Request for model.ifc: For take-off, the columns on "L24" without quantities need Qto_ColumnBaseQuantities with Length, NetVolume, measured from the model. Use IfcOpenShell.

First a look at what the model holds.

```python
import ifcopenshell
import ifcopenshell.util.element
import ifcopenshell.util.unit

model = ifcopenshell.open("model.ifc")
print(model.schema)
for unit_type in ("LENGTHUNIT", "AREAUNIT", "VOLUMEUNIT"):
    print(unit_type, ifcopenshell.util.unit.calculate_unit_scale(model, unit_type))
storey = next(s for s in model.by_type("IfcBuildingStorey") if s.Name == "L24")
columns = [e for e in ifcopenshell.util.element.get_decomposition(storey) if e.is_a("IfcColumn")]
for e in sorted(columns, key=lambda e: e.id()):
    print(e.id(), e.is_a(), e.Name, list(ifcopenshell.util.element.get_psets(e, qtos_only=True)), sep=" | ")
```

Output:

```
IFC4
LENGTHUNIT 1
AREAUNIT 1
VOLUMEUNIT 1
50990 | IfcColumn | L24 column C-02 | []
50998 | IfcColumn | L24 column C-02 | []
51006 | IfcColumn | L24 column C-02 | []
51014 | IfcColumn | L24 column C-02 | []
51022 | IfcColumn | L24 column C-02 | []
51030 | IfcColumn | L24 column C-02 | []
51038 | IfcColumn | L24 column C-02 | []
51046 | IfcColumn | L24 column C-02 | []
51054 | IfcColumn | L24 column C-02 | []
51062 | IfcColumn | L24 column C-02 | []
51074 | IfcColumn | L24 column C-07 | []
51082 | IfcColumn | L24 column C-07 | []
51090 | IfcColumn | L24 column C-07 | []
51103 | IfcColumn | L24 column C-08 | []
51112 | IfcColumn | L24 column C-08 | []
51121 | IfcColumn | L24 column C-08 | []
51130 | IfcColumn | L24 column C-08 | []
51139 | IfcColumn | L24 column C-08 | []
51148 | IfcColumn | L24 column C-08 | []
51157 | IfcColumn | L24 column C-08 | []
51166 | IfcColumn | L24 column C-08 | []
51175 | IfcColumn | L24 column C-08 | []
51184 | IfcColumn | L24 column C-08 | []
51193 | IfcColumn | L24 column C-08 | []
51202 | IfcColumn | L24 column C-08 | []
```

```python
import ifcopenshell
import ifcopenshell.api.pset
import ifcopenshell.geom
import ifcopenshell.util.element
import ifcopenshell.util.shape
import ifcopenshell.util.unit

model = ifcopenshell.open("model.ifc")
unit_scale = ifcopenshell.util.unit.calculate_unit_scale(model)
volume_scale = ifcopenshell.util.unit.calculate_unit_scale(model, "VOLUMEUNIT")
settings = ifcopenshell.geom.settings()

storey = next(s for s in model.by_type("IfcBuildingStorey") if s.Name == "L24")
columns = [e for e in ifcopenshell.util.element.get_decomposition(storey) if e.is_a("IfcColumn")]

for e in sorted(columns, key=lambda e: e.id()):
    if ifcopenshell.util.element.get_psets(e, qtos_only=True, should_inherit=False):
        continue
    # Geometry comes back in metres, in the element's own axes.
    shape = ifcopenshell.geom.create_shape(settings, e)
    values = {
        "Length": ifcopenshell.util.shape.get_z(shape.geometry) / unit_scale,
        "NetVolume": ifcopenshell.util.shape.get_volume(shape.geometry) / volume_scale,
    }
    qto = ifcopenshell.api.pset.add_qto(model, product=e, name="Qto_ColumnBaseQuantities")
    ifcopenshell.api.pset.edit_qto(model, qto=qto, properties=values)
    print(e.id(), {k: round(v, 3) for k, v in values.items()})

model.write("model_updated.ifc")
```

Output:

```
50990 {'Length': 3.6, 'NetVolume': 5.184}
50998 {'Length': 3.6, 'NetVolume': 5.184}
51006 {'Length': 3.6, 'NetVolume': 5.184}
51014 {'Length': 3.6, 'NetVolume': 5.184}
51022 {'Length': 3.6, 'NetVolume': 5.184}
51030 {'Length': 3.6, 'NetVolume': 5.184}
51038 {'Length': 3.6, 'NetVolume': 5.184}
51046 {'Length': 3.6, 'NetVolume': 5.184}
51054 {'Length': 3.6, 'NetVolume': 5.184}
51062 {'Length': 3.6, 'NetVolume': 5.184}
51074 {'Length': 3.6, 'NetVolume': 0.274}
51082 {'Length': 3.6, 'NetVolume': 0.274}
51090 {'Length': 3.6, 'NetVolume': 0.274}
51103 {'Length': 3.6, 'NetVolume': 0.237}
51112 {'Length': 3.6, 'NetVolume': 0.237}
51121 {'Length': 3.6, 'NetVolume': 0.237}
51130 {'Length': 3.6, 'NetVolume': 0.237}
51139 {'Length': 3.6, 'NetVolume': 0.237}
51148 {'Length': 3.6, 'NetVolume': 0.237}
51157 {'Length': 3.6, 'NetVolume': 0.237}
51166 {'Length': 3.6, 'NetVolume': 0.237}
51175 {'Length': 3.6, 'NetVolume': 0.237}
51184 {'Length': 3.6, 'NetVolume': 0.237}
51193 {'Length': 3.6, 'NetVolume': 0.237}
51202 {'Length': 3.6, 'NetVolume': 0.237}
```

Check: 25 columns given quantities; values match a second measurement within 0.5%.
